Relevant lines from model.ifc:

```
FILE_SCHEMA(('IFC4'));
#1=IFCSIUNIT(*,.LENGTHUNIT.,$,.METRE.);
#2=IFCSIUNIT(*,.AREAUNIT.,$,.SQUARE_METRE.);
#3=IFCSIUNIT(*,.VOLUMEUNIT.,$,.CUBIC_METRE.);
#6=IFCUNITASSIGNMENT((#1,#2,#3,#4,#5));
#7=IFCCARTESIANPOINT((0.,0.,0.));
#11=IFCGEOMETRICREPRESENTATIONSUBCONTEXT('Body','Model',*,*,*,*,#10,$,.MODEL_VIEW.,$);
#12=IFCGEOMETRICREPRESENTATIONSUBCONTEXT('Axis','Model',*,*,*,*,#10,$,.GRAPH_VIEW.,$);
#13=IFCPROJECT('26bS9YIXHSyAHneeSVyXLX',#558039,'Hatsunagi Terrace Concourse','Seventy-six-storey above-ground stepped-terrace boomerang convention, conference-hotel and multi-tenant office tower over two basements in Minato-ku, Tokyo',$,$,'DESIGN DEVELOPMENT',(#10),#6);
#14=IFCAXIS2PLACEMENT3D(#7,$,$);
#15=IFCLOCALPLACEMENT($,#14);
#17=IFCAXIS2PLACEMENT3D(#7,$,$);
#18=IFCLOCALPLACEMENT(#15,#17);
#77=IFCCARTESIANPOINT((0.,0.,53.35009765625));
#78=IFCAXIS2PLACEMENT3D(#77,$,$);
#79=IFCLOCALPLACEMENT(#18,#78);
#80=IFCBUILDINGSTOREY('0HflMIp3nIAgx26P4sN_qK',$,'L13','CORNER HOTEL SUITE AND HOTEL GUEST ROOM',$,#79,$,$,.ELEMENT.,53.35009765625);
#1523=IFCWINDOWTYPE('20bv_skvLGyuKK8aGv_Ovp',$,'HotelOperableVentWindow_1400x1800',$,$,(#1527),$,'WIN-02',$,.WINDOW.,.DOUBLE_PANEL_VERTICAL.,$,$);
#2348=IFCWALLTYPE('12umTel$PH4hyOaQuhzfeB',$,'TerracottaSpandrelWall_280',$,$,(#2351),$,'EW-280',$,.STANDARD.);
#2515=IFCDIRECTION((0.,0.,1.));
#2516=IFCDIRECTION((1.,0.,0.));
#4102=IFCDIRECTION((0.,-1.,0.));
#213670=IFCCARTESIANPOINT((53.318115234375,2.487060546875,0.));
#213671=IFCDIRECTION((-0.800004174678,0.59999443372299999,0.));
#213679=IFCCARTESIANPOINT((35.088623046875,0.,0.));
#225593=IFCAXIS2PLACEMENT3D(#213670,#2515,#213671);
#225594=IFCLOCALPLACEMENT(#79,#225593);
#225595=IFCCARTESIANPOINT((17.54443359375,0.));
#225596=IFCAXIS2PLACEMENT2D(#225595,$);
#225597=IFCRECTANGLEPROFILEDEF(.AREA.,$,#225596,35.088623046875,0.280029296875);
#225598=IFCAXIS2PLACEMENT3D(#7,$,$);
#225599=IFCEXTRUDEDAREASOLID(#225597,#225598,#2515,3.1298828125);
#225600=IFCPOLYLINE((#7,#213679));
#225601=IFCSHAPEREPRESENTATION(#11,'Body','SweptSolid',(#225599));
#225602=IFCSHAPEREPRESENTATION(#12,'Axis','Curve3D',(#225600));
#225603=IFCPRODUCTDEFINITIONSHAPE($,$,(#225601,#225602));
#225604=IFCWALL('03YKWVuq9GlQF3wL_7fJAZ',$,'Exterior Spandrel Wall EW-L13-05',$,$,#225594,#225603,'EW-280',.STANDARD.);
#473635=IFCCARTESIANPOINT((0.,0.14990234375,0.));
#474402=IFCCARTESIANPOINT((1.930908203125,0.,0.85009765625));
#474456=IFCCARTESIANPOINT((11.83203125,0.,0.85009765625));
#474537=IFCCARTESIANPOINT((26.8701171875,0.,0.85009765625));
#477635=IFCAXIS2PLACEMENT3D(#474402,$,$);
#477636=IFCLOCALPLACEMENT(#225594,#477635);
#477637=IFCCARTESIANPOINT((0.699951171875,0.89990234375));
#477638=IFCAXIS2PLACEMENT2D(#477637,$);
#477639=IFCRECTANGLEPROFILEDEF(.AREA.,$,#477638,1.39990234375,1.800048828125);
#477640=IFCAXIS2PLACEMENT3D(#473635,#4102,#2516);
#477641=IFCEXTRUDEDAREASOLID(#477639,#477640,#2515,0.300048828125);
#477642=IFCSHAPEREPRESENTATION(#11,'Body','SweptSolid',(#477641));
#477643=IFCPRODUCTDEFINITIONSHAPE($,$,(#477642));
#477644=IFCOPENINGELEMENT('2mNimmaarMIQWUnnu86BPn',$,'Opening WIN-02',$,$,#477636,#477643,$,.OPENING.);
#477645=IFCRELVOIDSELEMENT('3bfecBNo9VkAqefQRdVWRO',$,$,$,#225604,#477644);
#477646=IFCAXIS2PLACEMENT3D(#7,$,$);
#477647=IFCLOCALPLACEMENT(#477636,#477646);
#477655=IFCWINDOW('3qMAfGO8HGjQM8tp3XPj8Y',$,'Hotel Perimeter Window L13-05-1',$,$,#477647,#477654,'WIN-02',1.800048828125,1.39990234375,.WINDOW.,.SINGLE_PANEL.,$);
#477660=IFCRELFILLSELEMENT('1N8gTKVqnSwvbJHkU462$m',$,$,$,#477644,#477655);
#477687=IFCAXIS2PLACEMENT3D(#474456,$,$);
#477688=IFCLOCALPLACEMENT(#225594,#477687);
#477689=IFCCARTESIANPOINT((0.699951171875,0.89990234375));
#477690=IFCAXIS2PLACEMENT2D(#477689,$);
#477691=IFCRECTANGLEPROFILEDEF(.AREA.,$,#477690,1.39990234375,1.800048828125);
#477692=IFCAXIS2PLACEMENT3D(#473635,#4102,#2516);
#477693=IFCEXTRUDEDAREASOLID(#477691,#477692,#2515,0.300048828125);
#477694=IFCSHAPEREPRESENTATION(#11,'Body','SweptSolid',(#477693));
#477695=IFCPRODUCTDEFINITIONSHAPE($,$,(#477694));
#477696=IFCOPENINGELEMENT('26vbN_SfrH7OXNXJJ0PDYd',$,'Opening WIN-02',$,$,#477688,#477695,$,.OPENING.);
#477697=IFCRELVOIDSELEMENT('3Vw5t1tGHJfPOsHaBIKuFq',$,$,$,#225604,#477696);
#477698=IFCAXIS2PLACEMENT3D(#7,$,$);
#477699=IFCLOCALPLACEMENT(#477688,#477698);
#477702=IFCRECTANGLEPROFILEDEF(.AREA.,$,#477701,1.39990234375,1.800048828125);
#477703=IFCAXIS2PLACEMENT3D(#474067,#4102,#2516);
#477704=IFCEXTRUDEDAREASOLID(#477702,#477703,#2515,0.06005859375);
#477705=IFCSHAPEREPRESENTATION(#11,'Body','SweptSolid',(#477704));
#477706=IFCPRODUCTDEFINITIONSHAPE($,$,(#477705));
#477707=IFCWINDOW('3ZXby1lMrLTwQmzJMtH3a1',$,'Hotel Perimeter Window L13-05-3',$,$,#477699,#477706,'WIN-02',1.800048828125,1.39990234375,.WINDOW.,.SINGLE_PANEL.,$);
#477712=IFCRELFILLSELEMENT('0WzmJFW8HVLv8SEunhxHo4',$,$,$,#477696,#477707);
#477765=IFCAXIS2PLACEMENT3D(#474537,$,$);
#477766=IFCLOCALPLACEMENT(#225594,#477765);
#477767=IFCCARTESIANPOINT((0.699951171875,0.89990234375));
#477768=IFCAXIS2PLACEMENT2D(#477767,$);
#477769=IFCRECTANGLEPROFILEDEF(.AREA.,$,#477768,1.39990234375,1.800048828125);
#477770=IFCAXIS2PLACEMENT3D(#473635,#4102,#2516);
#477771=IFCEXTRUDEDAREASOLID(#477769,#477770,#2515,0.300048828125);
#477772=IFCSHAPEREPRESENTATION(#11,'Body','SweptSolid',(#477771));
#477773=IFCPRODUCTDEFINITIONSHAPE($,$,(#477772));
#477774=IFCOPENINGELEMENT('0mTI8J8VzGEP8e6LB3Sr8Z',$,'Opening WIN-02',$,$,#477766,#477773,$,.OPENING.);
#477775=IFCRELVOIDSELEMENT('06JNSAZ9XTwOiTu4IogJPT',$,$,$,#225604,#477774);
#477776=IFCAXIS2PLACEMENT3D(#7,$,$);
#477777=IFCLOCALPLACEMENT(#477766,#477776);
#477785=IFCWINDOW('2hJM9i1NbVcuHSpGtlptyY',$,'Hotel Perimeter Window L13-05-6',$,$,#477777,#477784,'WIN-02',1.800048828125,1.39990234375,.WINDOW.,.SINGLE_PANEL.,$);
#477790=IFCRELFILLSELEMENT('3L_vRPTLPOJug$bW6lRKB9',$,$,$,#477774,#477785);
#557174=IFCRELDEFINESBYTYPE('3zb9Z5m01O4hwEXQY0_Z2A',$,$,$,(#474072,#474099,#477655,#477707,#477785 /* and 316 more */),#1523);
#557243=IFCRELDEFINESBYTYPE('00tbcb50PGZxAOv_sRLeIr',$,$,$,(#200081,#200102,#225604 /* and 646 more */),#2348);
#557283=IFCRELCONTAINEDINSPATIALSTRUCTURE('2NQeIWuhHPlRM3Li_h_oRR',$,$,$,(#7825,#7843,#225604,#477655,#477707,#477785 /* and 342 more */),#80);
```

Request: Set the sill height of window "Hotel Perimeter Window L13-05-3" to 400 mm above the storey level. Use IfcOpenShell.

```python
import numpy as np
import ifcopenshell
import ifcopenshell.api.geometry
import ifcopenshell.geom
import ifcopenshell.util.element
import ifcopenshell.util.placement
import ifcopenshell.util.shape
import ifcopenshell.util.unit

model = ifcopenshell.open("model.ifc")
unit_scale = ifcopenshell.util.unit.calculate_unit_scale(model)

window = model.by_guid("3ZXby1lMrLTwQmzJMtH3a1")
opening = window.FillsVoids[0].RelatingOpeningElement
storey = ifcopenshell.util.element.get_container(window, ifc_class="IfcBuildingStorey")
level = ifcopenshell.util.placement.get_local_placement(storey.ObjectPlacement)[2, 3]

# The opening's origin need not be at the sill, so measure its lowest point.
shape = ifcopenshell.geom.create_shape(ifcopenshell.geom.settings(), opening)
bottom = ifcopenshell.util.shape.get_shape_bottom_elevation(shape, shape.geometry) / unit_scale
dz = level + 0.4 / unit_scale - bottom

shift = np.array([0.0, 0.0, dz])
# The window is placed relative to its opening, so it follows when the opening moves.
matrix = ifcopenshell.util.placement.get_local_placement(opening.ObjectPlacement)
matrix[:3, 3] += shift
ifcopenshell.api.geometry.edit_object_placement(
    model, product=opening, matrix=matrix, is_si=False, should_transform_children=True
)

print(f"moved by {dz * unit_scale:+.3f} m")

model.write("model_updated.ifc")
```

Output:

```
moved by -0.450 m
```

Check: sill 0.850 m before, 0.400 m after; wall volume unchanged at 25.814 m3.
